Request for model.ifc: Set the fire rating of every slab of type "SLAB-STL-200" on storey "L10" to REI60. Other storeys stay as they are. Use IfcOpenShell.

First a look at what the model holds.

```python
import ifcopenshell
import ifcopenshell.util.element

model = ifcopenshell.open("model.ifc")
print(model.schema)
storey = next(s for s in model.by_type("IfcBuildingStorey") if s.Name == "L10")
slabs = [e for e in ifcopenshell.util.element.get_decomposition(storey) if e.is_a("IfcSlab")]
seen = {}
for e in slabs:
    element_type = ifcopenshell.util.element.get_type(e)
    key = (element_type.Name if element_type != e and element_type else None, ifcopenshell.util.element.get_pset(e, "Pset_SlabCommon", "FireRating"))
    seen[key] = seen.get(key, 0) + 1
for (name, value), count in sorted(seen.items(), key=str):
    print(count, "x", name, "|", value)
```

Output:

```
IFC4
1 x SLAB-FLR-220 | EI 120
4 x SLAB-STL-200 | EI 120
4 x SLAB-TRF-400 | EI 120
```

```python
import ifcopenshell
import ifcopenshell.api.pset
import ifcopenshell.util.element

model = ifcopenshell.open("model.ifc")

storey = next(s for s in model.by_type("IfcBuildingStorey") if s.Name == "L10")
slabs = [e for e in ifcopenshell.util.element.get_decomposition(storey) if e.is_a("IfcSlab")]

count = 0
for e in slabs:
    element_type = ifcopenshell.util.element.get_type(e)
    if element_type in (None, e) or element_type.Name != "SLAB-STL-200":
        continue
    found = ifcopenshell.util.element.get_pset(e, "Pset_SlabCommon", should_inherit=False)
    if found:
        pset = model.by_id(found["id"])
        if len(ifcopenshell.util.element.get_elements_by_pset(pset)) > 1:
            pset = ifcopenshell.api.pset.unshare_pset(model, products=[e], pset=pset)[0]
    else:
        pset = ifcopenshell.api.pset.add_pset(model, product=e, name="Pset_SlabCommon")
    ifcopenshell.api.pset.edit_pset(model, pset=pset, properties={"FireRating": "REI60"})
    count += 1

print(count, "slabs updated")

model.write("model_rev.ifc")
```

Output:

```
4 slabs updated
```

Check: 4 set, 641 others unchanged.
